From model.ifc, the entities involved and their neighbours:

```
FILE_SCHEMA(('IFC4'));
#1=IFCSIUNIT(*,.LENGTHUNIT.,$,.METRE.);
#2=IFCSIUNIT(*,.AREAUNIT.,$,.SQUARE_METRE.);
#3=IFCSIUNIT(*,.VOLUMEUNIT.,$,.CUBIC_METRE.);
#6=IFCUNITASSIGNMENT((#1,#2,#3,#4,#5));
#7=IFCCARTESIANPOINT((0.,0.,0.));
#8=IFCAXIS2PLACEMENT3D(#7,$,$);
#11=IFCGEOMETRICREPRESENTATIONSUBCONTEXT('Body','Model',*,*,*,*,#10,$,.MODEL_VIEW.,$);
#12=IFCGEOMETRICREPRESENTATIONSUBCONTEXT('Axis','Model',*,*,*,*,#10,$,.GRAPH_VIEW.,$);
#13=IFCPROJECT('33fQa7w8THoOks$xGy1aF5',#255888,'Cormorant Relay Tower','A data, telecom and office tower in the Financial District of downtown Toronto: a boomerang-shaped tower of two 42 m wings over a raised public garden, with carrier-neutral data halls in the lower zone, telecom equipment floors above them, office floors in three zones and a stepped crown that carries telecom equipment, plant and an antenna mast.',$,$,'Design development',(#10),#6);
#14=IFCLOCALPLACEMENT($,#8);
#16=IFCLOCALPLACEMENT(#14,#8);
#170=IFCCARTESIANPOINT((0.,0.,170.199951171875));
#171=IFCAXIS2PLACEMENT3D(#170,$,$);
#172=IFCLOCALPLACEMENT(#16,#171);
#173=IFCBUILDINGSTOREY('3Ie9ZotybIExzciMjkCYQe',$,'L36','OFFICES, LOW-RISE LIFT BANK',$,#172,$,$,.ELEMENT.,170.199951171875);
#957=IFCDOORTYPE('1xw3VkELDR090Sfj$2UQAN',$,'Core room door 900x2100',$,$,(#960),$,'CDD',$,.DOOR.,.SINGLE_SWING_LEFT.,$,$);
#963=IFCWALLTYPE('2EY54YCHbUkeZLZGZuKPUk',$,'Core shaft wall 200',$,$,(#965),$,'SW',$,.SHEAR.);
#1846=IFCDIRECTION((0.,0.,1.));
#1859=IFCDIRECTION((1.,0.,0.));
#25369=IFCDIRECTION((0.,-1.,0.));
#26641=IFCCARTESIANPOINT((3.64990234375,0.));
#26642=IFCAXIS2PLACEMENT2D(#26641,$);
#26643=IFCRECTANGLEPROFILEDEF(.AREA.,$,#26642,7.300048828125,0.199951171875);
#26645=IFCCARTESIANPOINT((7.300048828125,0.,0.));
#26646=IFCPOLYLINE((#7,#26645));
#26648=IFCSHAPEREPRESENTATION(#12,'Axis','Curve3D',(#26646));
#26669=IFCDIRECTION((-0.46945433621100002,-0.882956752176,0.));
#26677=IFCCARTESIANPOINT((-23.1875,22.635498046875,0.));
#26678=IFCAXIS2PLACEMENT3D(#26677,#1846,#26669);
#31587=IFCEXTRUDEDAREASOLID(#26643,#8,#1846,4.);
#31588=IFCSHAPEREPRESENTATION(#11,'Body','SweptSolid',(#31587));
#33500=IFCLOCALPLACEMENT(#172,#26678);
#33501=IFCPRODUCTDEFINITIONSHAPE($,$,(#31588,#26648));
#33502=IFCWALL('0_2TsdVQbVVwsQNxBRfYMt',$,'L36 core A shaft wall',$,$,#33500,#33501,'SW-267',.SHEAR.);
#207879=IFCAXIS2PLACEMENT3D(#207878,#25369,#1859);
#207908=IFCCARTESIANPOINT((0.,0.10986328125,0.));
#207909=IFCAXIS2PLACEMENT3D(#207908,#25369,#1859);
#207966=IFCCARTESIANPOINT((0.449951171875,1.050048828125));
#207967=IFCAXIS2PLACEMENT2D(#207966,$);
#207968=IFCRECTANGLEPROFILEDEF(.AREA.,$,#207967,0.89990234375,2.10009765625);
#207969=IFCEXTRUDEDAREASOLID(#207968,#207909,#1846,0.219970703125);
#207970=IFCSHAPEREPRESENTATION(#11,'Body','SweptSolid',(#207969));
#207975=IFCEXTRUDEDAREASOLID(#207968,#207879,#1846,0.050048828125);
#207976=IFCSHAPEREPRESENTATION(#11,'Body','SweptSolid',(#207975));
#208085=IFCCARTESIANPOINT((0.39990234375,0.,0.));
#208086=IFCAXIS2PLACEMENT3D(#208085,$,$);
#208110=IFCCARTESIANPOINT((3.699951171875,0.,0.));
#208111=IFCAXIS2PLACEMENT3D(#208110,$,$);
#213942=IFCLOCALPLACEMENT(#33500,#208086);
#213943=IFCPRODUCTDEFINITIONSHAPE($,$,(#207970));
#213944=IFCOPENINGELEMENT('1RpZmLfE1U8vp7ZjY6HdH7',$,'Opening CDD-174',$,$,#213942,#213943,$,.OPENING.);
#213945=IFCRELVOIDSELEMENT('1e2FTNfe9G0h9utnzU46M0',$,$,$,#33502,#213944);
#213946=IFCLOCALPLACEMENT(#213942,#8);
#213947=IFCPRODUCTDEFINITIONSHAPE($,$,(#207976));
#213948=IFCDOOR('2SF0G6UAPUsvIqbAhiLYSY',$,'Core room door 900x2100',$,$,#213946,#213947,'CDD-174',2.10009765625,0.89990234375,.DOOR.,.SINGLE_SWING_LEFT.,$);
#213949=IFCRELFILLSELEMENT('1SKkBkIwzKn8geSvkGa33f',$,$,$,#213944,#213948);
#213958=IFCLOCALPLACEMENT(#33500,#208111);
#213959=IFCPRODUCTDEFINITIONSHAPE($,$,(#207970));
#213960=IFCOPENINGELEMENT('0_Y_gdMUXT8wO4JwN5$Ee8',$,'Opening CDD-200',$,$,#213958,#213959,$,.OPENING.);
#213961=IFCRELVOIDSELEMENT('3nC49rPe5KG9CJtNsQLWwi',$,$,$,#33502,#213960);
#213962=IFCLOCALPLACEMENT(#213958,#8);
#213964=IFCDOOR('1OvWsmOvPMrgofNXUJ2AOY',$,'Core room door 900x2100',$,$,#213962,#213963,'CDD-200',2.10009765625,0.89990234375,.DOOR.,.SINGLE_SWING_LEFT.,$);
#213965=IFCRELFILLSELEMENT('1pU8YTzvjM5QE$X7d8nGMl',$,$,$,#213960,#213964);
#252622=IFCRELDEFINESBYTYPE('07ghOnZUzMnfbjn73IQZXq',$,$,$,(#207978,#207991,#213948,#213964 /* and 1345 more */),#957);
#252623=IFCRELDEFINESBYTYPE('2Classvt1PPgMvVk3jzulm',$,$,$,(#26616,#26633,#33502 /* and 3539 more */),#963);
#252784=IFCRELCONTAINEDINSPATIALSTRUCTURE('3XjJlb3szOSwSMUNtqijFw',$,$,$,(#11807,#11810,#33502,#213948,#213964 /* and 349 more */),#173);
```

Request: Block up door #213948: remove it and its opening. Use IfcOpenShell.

```python
import ifcopenshell
import ifcopenshell.api.feature
import ifcopenshell.api.root
import ifcopenshell.geom
import ifcopenshell.util.shape

model = ifcopenshell.open("model.ifc")
settings = ifcopenshell.geom.settings()


def volume(element):
    """Net volume in cubic metres, openings subtracted."""
    shape = ifcopenshell.geom.create_shape(settings, element)
    return ifcopenshell.util.shape.get_volume(shape.geometry)


door = model.by_id(213948)
opening = door.FillsVoids[0].RelatingOpeningElement
wall = opening.VoidsElements[0].RelatingBuildingElement
before = volume(wall)

ifcopenshell.api.root.remove_product(model, product=door)
ifcopenshell.api.feature.remove_feature(model, feature=opening)

after = volume(wall)

print(f"wall volume {before:.3f} -> {after:.3f} m3")

model.write("model_updated.ifc")
```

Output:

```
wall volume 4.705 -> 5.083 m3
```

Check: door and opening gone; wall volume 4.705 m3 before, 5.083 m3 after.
